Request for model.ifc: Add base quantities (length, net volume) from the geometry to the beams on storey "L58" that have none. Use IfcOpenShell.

First a look at what the model holds.

```python
import ifcopenshell
import ifcopenshell.util.element
import ifcopenshell.util.unit

model = ifcopenshell.open("model.ifc")
print(model.schema)
for unit_type in ("LENGTHUNIT", "AREAUNIT", "VOLUMEUNIT"):
    print(unit_type, ifcopenshell.util.unit.calculate_unit_scale(model, unit_type))
storey = next(s for s in model.by_type("IfcBuildingStorey") if s.Name == "L58")
beams = [e for e in ifcopenshell.util.element.get_decomposition(storey) if e.is_a("IfcBeam")]
for e in sorted(beams, key=lambda e: e.id()):
    print(e.id(), e.is_a(), e.Name, list(ifcopenshell.util.element.get_psets(e, qtos_only=True)), sep=" | ")
```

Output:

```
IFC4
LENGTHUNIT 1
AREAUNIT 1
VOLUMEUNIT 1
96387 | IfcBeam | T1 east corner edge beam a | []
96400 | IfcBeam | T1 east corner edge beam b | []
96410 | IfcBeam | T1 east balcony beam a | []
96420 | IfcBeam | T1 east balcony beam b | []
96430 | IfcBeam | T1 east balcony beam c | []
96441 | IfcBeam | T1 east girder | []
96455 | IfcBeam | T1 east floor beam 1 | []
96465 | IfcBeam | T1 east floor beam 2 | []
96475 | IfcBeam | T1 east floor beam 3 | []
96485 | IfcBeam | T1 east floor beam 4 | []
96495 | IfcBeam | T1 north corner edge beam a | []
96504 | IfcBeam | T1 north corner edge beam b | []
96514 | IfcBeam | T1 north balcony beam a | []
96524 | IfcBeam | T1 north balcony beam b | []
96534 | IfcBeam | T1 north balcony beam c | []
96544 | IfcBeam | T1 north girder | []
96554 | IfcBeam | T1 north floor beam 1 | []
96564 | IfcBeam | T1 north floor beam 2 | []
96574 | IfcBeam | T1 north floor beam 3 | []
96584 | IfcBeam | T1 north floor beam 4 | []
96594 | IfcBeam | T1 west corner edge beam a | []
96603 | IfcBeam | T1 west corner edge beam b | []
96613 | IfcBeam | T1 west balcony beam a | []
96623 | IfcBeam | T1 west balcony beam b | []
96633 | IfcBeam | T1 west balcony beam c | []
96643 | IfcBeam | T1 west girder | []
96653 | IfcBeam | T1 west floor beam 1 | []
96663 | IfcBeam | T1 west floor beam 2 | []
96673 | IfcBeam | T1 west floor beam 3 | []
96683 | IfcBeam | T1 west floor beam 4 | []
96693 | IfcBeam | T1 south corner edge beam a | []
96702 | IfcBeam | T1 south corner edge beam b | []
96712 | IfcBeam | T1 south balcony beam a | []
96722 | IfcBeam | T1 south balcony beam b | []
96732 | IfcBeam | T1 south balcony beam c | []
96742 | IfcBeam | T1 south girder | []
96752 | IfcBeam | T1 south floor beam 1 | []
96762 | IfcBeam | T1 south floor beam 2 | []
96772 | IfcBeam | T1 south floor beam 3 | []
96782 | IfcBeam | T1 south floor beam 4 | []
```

```python
import ifcopenshell
import ifcopenshell.api.pset
import ifcopenshell.geom
import ifcopenshell.util.element
import ifcopenshell.util.shape
import ifcopenshell.util.unit

model = ifcopenshell.open("model.ifc")
unit_scale = ifcopenshell.util.unit.calculate_unit_scale(model)
volume_scale = ifcopenshell.util.unit.calculate_unit_scale(model, "VOLUMEUNIT")
settings = ifcopenshell.geom.settings()

storey = next(s for s in model.by_type("IfcBuildingStorey") if s.Name == "L58")
beams = [e for e in ifcopenshell.util.element.get_decomposition(storey) if e.is_a("IfcBeam")]

for e in sorted(beams, key=lambda e: e.id()):
    if ifcopenshell.util.element.get_psets(e, qtos_only=True, should_inherit=False):
        continue
    # Geometry comes back in metres, in the element's own axes.
    shape = ifcopenshell.geom.create_shape(settings, e)
    values = {
        "Length": ifcopenshell.util.shape.get_max_xyz(shape.geometry) / unit_scale,
        "NetVolume": ifcopenshell.util.shape.get_volume(shape.geometry) / volume_scale,
    }
    qto = ifcopenshell.api.pset.add_qto(model, product=e, name="Qto_BeamBaseQuantities")
    ifcopenshell.api.pset.edit_qto(model, qto=qto, properties=values)
    print(e.id(), {k: round(v, 3) for k, v in values.items()})

model.write("model_v2.ifc")
```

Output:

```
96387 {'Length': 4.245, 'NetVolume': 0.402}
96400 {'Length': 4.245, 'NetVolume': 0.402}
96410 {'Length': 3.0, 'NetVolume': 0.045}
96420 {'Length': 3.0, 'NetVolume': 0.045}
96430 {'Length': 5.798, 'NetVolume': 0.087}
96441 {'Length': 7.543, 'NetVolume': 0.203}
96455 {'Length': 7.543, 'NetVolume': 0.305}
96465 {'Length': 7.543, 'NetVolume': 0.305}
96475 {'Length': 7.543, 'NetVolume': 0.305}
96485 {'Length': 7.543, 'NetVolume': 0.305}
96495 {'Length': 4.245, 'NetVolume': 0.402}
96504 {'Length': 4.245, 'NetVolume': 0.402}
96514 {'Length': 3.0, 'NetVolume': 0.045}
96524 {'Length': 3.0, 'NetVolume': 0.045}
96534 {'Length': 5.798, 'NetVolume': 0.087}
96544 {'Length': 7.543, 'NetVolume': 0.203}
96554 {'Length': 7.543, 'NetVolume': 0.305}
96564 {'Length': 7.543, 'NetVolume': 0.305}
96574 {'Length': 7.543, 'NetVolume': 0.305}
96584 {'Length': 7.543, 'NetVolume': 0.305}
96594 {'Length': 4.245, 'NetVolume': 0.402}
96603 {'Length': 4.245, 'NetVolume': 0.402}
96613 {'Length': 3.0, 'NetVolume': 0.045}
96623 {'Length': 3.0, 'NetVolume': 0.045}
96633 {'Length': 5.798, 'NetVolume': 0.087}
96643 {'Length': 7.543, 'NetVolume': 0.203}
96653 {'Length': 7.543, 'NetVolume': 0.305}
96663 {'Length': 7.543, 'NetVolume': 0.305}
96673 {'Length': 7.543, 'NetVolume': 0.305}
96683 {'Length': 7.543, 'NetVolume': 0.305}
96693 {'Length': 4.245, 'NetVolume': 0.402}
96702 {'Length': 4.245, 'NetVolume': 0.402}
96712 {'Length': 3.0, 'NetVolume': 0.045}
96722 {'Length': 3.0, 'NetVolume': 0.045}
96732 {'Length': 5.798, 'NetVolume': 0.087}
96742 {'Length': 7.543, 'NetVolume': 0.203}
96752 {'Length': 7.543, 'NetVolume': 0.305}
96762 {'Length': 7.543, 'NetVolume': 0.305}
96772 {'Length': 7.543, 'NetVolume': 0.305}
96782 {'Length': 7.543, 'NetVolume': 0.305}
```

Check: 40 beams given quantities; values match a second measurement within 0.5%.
